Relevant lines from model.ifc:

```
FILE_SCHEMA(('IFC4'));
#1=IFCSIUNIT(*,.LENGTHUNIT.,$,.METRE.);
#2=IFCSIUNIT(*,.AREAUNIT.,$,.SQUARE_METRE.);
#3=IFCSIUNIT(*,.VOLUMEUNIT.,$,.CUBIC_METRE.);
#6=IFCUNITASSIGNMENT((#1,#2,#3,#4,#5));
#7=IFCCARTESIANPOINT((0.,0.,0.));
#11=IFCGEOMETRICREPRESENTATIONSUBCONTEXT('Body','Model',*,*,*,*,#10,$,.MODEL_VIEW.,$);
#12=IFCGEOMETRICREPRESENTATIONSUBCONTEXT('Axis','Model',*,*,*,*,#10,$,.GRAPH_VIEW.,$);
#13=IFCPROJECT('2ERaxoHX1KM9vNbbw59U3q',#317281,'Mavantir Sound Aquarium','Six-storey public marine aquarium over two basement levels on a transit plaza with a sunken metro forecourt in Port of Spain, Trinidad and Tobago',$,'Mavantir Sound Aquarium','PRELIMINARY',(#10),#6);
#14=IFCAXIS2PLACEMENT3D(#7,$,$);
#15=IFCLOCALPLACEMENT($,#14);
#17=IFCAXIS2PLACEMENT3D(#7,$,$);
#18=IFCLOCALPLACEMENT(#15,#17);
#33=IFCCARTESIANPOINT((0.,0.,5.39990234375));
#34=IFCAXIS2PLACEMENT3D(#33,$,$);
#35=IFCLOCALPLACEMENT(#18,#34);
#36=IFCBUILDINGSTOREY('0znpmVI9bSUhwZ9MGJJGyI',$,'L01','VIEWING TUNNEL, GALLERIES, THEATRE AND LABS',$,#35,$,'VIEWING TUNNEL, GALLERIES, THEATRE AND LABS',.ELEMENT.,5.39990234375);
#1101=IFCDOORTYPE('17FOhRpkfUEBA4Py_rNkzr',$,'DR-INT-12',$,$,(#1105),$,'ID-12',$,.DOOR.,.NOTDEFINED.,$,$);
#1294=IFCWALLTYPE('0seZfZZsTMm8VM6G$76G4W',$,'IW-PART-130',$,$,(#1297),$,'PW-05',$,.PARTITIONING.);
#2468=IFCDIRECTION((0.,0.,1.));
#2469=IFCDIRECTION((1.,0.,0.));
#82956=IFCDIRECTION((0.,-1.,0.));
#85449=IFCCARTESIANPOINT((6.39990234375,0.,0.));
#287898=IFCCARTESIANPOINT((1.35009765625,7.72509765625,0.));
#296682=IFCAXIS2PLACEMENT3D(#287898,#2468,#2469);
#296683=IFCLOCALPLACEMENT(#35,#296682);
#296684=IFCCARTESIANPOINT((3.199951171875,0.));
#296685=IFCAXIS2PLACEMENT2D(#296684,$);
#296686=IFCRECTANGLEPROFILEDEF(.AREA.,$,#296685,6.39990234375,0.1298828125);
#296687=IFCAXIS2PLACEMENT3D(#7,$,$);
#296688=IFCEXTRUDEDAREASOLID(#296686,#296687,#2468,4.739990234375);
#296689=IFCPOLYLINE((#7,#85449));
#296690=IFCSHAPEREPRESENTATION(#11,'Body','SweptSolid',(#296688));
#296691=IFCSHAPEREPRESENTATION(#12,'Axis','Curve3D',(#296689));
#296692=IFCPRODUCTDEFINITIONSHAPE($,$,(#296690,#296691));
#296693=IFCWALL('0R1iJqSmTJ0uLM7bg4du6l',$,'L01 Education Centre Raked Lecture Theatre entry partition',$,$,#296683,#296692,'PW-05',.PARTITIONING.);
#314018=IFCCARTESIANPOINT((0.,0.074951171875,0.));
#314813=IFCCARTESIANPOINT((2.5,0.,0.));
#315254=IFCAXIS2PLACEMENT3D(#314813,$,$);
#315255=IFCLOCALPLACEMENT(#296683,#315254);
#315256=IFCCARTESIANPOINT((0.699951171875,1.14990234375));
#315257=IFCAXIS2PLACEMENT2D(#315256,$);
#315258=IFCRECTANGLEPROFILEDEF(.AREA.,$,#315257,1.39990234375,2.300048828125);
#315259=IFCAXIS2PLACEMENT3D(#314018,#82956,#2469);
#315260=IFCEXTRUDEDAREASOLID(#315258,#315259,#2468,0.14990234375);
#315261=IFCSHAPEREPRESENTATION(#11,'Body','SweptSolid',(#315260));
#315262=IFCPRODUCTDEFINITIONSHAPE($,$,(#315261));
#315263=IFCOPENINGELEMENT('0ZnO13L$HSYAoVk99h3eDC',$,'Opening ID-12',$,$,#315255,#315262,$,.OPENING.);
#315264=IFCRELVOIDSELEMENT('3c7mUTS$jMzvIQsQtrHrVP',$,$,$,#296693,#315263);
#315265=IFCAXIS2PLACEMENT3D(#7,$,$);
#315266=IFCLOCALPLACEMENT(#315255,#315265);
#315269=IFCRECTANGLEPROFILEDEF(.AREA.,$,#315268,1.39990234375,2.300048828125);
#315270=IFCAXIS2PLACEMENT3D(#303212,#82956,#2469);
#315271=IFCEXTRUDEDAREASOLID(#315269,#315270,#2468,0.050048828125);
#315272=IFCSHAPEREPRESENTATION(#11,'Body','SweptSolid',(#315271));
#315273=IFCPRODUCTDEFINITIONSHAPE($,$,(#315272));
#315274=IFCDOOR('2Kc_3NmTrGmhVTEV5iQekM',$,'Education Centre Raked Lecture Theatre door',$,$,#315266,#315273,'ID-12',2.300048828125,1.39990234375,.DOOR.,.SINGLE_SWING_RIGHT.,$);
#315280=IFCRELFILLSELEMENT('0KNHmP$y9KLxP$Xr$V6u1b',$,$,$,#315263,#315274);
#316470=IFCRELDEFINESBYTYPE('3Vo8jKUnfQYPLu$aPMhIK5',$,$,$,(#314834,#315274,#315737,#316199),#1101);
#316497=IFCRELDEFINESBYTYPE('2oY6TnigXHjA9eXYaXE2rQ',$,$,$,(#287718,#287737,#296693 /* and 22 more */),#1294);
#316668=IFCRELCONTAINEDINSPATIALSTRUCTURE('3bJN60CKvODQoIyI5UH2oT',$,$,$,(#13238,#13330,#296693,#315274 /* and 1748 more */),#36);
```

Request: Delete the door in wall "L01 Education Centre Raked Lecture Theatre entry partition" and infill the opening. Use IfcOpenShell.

```python
import ifcopenshell
import ifcopenshell.api.feature
import ifcopenshell.api.root
import ifcopenshell.geom
import ifcopenshell.util.shape

model = ifcopenshell.open("model.ifc")
settings = ifcopenshell.geom.settings()


def volume(element):
    """Net volume in cubic metres, openings subtracted."""
    shape = ifcopenshell.geom.create_shape(settings, element)
    return ifcopenshell.util.shape.get_volume(shape.geometry)


door = model.by_guid("2Kc_3NmTrGmhVTEV5iQekM")
opening = door.FillsVoids[0].RelatingOpeningElement
wall = opening.VoidsElements[0].RelatingBuildingElement
before = volume(wall)

ifcopenshell.api.root.remove_product(model, product=door)
ifcopenshell.api.feature.remove_feature(model, feature=opening)

after = volume(wall)

print(f"wall volume {before:.3f} -> {after:.3f} m3")

model.write("model_v2.ifc")
```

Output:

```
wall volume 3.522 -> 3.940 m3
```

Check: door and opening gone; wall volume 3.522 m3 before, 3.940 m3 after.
